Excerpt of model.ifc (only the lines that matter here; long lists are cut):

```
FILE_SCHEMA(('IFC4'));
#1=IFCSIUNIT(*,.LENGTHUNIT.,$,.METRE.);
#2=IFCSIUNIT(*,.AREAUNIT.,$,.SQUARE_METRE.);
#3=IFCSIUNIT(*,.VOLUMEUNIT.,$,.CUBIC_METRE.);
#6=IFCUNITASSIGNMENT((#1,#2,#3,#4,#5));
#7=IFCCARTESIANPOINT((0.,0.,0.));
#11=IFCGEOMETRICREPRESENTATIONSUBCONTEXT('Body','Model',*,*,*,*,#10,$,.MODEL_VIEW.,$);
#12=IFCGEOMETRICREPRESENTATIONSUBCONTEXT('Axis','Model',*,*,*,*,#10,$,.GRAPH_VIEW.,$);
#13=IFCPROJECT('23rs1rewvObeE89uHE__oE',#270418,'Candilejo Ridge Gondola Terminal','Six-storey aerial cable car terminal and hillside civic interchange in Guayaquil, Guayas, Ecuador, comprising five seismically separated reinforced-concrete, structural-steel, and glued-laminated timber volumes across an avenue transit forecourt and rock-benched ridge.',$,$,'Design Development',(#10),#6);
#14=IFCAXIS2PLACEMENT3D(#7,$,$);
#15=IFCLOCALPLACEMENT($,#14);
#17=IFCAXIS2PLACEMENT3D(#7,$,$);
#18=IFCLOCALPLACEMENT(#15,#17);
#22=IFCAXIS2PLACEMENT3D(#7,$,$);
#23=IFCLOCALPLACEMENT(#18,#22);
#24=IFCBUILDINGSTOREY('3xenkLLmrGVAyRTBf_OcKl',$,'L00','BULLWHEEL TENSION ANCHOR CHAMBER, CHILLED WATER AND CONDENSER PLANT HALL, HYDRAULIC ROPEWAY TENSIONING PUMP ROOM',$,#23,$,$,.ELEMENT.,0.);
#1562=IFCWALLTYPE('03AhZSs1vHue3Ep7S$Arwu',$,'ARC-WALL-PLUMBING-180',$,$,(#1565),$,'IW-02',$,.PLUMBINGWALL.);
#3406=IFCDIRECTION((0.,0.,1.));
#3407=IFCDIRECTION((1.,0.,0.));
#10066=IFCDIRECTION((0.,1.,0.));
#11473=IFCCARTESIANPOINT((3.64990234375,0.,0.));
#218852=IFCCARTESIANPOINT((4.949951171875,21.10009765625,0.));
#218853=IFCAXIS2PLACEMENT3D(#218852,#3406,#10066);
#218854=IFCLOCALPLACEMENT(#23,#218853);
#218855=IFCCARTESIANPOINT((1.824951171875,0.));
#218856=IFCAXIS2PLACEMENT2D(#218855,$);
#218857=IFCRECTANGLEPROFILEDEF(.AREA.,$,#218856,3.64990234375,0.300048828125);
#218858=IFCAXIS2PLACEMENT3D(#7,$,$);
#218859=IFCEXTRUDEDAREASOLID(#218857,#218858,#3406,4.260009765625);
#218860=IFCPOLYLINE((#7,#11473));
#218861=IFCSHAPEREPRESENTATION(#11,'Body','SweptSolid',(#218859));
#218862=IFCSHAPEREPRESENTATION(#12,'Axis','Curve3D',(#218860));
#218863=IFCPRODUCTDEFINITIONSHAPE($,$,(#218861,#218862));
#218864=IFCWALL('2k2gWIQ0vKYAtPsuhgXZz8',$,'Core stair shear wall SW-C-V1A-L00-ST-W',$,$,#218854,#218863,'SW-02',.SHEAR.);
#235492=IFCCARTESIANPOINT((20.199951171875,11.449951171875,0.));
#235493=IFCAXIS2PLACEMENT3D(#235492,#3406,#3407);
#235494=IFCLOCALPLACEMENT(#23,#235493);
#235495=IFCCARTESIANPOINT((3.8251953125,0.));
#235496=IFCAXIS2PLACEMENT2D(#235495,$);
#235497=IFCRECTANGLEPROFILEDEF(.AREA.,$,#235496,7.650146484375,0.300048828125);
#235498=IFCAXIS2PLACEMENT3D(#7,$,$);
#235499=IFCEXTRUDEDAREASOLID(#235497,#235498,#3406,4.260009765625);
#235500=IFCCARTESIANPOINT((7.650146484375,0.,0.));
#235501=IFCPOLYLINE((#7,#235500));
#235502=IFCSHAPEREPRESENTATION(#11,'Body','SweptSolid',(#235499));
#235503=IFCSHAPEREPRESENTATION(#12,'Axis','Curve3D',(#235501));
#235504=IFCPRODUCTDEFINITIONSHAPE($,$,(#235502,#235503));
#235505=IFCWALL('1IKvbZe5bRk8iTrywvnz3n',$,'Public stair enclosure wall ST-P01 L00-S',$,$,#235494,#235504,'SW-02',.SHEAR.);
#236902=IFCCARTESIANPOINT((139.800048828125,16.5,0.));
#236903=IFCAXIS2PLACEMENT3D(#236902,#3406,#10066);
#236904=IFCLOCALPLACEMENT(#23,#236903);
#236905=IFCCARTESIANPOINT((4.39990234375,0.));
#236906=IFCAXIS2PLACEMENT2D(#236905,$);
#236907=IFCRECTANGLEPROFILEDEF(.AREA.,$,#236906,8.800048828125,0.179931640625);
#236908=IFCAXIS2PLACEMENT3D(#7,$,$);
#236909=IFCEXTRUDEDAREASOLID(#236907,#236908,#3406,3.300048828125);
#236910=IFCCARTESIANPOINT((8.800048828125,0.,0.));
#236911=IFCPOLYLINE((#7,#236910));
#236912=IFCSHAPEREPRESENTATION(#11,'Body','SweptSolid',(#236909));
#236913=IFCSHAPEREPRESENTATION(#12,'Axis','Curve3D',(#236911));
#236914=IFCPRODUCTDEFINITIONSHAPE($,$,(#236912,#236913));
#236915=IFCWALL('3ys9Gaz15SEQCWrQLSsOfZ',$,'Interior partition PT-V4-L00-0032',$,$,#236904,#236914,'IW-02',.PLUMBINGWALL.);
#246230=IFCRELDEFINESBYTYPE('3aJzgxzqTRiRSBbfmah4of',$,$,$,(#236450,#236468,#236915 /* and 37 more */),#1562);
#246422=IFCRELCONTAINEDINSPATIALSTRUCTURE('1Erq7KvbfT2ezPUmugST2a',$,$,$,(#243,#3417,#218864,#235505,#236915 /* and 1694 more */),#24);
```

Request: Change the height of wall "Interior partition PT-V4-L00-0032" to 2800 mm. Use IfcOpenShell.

```python
import ifcopenshell
import ifcopenshell.geom
import ifcopenshell.util.representation
import ifcopenshell.util.shape

model = ifcopenshell.open("model.ifc")
settings = ifcopenshell.geom.settings()


def volume(element):
    """Net volume in cubic metres, openings subtracted."""
    shape = ifcopenshell.geom.create_shape(settings, element)
    return ifcopenshell.util.shape.get_volume(shape.geometry)


wall = model.by_id(236915)
before = volume(wall)

body = ifcopenshell.util.representation.get_representation(wall, "Model", "Body")
solid = body.Items[0]
old_height = solid.Depth
solid.Depth = 2.8
after = volume(wall)

print(f"height {old_height:g} -> {solid.Depth:g}, volume {before:.3f} -> {after:.3f} m3")

model.write("model_rev.ifc")
```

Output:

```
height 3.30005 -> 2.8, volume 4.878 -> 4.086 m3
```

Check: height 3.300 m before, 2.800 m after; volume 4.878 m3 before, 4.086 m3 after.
